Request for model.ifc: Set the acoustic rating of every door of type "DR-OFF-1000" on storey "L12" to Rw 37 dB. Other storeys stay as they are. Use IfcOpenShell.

First a look at what the model holds.

```python
import ifcopenshell
import ifcopenshell.util.element

model = ifcopenshell.open("model.ifc")
print(model.schema)
storey = next(s for s in model.by_type("IfcBuildingStorey") if s.Name == "L12")
doors = [e for e in ifcopenshell.util.element.get_decomposition(storey) if e.is_a("IfcDoor")]
seen = {}
for e in doors:
    element_type = ifcopenshell.util.element.get_type(e)
    key = (element_type.Name if element_type != e and element_type else None, ifcopenshell.util.element.get_pset(e, "Pset_DoorCommon", "AcousticRating"))
    seen[key] = seen.get(key, 0) + 1
for (name, value), count in sorted(seen.items(), key=str):
    print(count, "x", name, "|", value)
```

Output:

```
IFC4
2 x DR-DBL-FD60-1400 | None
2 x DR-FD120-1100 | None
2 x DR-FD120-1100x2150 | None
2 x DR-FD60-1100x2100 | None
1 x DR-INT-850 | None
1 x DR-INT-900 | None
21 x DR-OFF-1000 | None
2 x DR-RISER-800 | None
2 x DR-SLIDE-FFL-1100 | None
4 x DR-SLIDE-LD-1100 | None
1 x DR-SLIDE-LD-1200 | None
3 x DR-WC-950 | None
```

```python
import ifcopenshell
import ifcopenshell.api.pset
import ifcopenshell.util.element

model = ifcopenshell.open("model.ifc")

storey = next(s for s in model.by_type("IfcBuildingStorey") if s.Name == "L12")
doors = [e for e in ifcopenshell.util.element.get_decomposition(storey) if e.is_a("IfcDoor")]

count = 0
for e in doors:
    element_type = ifcopenshell.util.element.get_type(e)
    if element_type in (None, e) or element_type.Name != "DR-OFF-1000":
        continue
    found = ifcopenshell.util.element.get_pset(e, "Pset_DoorCommon", should_inherit=False)
    if found:
        pset = model.by_id(found["id"])
        if len(ifcopenshell.util.element.get_elements_by_pset(pset)) > 1:
            pset = ifcopenshell.api.pset.unshare_pset(model, products=[e], pset=pset)[0]
    else:
        pset = ifcopenshell.api.pset.add_pset(model, product=e, name="Pset_DoorCommon")
    ifcopenshell.api.pset.edit_pset(model, pset=pset, properties={"AcousticRating": "Rw 37 dB"})
    count += 1

print(count, "doors updated")

model.write("model_v2.ifc")
```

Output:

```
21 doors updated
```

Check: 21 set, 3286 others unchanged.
